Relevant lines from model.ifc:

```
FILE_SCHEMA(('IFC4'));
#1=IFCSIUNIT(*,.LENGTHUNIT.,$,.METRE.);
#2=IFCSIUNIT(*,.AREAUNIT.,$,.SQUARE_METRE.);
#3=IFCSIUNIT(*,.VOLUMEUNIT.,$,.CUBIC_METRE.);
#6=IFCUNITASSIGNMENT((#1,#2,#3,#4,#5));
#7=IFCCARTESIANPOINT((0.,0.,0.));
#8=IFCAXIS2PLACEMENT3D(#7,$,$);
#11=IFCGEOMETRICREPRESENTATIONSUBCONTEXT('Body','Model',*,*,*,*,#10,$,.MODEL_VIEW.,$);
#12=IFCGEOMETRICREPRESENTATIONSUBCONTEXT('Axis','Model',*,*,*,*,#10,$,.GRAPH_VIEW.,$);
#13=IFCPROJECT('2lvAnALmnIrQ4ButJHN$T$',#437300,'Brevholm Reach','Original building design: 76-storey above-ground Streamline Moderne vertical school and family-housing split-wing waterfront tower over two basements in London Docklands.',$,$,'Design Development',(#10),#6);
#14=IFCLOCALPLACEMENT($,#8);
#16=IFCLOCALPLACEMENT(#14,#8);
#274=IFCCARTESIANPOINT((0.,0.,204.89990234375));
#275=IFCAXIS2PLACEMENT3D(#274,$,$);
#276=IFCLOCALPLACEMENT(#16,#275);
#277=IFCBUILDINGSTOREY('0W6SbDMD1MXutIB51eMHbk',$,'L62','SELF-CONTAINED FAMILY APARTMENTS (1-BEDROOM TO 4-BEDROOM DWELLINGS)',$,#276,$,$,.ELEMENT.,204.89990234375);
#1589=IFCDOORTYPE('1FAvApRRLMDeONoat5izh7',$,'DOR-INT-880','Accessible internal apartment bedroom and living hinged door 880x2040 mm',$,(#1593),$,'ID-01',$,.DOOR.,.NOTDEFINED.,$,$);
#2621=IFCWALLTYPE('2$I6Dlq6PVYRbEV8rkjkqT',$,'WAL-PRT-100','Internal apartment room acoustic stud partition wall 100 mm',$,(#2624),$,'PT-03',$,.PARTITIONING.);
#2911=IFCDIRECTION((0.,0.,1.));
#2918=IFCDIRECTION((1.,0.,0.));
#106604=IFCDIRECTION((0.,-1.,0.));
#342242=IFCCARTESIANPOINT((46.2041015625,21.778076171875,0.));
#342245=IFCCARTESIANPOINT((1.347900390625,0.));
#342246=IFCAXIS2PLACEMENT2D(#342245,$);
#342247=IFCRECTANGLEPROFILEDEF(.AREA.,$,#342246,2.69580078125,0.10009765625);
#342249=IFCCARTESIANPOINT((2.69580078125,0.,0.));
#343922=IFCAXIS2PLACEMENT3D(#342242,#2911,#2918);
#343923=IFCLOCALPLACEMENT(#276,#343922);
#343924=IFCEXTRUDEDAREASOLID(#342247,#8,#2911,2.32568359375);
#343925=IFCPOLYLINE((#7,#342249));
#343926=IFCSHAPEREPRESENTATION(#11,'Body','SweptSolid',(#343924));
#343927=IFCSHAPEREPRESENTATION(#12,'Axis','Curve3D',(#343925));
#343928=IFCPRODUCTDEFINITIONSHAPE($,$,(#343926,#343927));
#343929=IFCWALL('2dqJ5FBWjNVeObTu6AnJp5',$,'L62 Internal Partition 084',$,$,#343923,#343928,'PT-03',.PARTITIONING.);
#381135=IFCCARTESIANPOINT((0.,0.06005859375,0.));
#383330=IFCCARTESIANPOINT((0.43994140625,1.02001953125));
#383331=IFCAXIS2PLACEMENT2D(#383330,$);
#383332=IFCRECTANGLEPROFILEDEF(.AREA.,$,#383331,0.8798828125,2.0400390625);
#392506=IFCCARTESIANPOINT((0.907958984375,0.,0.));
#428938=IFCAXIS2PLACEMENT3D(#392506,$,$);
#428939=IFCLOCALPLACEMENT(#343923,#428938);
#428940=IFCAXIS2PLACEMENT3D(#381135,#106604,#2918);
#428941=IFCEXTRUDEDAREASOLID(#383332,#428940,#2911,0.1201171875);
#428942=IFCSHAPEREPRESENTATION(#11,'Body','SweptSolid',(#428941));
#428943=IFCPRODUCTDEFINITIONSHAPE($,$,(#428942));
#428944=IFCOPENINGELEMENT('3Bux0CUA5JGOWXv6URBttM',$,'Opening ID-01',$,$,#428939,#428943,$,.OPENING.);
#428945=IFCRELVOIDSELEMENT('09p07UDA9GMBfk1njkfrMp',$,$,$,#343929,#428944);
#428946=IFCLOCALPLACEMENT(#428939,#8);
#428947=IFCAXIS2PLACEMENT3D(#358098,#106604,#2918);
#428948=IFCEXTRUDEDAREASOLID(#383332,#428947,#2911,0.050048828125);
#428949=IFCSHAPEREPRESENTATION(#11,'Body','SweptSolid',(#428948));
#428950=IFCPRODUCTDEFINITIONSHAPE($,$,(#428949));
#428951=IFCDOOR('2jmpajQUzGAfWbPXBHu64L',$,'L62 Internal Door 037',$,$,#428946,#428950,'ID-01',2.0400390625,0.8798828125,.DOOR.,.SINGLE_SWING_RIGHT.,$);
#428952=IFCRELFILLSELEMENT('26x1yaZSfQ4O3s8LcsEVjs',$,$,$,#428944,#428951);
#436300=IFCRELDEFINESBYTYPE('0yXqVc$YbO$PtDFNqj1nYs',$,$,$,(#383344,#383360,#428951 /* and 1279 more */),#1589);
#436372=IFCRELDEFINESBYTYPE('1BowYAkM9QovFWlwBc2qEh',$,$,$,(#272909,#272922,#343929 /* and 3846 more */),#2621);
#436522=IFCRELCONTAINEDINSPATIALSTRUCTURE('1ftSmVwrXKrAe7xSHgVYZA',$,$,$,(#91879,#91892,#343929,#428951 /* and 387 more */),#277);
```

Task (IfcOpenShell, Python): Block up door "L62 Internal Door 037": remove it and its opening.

```python
import ifcopenshell
import ifcopenshell.api.feature
import ifcopenshell.api.root
import ifcopenshell.geom
import ifcopenshell.util.shape

model = ifcopenshell.open("model.ifc")
settings = ifcopenshell.geom.settings()


def volume(element):
    """Net volume in cubic metres, openings subtracted."""
    shape = ifcopenshell.geom.create_shape(settings, element)
    return ifcopenshell.util.shape.get_volume(shape.geometry)


door = model.by_guid("2jmpajQUzGAfWbPXBHu64L")
opening = door.FillsVoids[0].RelatingOpeningElement
wall = opening.VoidsElements[0].RelatingBuildingElement
before = volume(wall)

ifcopenshell.api.root.remove_product(model, product=door)
ifcopenshell.api.feature.remove_feature(model, feature=opening)

after = volume(wall)

print(f"wall volume {before:.3f} -> {after:.3f} m3")

model.write("model_edited.ifc")
```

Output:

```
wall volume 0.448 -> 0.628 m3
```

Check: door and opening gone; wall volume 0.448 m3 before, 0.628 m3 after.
